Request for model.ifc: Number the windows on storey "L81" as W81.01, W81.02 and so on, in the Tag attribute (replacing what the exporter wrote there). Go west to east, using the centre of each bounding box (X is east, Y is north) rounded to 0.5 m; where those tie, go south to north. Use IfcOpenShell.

First a look at what the model holds.

```python
import ifcopenshell
import ifcopenshell.util.element
import ifcopenshell.util.placement

model = ifcopenshell.open("model.ifc")
print(model.schema)
storey = next(s for s in model.by_type("IfcBuildingStorey") if s.Name == "L81")
windows = [e for e in ifcopenshell.util.element.get_decomposition(storey) if e.is_a("IfcWindow")]
for e in sorted(windows, key=lambda e: e.id()):
    origin = ifcopenshell.util.placement.get_local_placement(e.ObjectPlacement)[:3, 3]
    print(e.id(), e.Tag, e.Name, origin.round(2) + 0.0, sep=" | ")
```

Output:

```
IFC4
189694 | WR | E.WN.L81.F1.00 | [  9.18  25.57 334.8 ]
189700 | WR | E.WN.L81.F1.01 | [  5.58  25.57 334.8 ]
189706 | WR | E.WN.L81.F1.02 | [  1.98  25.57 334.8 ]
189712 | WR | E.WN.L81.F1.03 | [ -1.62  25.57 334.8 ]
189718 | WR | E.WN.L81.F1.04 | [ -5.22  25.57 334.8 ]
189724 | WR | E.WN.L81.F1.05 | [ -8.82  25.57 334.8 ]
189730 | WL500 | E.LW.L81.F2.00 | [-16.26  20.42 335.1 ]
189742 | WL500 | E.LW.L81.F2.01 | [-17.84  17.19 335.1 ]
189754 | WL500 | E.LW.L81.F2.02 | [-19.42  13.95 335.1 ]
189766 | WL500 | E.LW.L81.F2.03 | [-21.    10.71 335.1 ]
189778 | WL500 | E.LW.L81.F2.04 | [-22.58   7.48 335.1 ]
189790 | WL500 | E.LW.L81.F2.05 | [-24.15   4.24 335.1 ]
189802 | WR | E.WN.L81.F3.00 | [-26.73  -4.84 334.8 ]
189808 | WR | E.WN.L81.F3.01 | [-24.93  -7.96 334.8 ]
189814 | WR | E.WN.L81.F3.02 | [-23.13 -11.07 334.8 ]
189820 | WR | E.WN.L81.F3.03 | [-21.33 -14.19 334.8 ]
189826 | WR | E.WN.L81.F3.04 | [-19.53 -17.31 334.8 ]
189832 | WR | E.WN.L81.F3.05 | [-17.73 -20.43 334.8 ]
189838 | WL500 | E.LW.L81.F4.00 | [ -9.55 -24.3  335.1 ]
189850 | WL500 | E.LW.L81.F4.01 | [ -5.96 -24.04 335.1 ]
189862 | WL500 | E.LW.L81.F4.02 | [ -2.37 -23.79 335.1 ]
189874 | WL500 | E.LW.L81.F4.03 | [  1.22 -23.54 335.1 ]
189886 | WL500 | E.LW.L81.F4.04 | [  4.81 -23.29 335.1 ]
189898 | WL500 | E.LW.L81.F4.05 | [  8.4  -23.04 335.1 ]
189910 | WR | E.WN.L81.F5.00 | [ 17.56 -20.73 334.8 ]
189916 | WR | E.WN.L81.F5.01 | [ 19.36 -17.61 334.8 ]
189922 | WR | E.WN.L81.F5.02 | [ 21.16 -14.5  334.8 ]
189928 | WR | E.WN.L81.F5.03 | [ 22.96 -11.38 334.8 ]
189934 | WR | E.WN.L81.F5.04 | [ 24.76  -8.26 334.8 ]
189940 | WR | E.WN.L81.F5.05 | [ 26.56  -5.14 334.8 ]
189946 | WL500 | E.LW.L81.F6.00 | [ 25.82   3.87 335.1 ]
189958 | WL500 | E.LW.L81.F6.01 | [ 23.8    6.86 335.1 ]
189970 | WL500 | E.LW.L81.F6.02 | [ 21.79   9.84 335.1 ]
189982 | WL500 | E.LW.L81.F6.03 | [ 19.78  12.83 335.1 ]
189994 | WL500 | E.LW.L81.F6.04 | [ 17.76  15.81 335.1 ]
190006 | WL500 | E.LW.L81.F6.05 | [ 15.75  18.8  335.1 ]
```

```python
import ifcopenshell
import ifcopenshell.geom
import ifcopenshell.util.element
import ifcopenshell.util.shape

model = ifcopenshell.open("model.ifc")
settings = ifcopenshell.geom.settings()
settings.set("use-world-coords", True)


def centre(element):
    shape = ifcopenshell.geom.create_shape(settings, element)
    return ifcopenshell.util.shape.get_bbox_centroid(shape.geometry)


storey = next(s for s in model.by_type("IfcBuildingStorey") if s.Name == "L81")
windows = [e for e in ifcopenshell.util.element.get_decomposition(storey) if e.is_a("IfcWindow")]

# Insertion points can sit at a corner or the storey origin, so sort by the geometry (in metres).
centres = {e: centre(e) for e in windows}
windows.sort(key=lambda e: (round(centres[e][0] / 0.5), centres[e][1]))

for i, e in enumerate(windows, start=1):
    number = f"W81.{i:02d}"
    e.Tag = number
    print(e.id(), number)

model.write("model_updated.ifc")
```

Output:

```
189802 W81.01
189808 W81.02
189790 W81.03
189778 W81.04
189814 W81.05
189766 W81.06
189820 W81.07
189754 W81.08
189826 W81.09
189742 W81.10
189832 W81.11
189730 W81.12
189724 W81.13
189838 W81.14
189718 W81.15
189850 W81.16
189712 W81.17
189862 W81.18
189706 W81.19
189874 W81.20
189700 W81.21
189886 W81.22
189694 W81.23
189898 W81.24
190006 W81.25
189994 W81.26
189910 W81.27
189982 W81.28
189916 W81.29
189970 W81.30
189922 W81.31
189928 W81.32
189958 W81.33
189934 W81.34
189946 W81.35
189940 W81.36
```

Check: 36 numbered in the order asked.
